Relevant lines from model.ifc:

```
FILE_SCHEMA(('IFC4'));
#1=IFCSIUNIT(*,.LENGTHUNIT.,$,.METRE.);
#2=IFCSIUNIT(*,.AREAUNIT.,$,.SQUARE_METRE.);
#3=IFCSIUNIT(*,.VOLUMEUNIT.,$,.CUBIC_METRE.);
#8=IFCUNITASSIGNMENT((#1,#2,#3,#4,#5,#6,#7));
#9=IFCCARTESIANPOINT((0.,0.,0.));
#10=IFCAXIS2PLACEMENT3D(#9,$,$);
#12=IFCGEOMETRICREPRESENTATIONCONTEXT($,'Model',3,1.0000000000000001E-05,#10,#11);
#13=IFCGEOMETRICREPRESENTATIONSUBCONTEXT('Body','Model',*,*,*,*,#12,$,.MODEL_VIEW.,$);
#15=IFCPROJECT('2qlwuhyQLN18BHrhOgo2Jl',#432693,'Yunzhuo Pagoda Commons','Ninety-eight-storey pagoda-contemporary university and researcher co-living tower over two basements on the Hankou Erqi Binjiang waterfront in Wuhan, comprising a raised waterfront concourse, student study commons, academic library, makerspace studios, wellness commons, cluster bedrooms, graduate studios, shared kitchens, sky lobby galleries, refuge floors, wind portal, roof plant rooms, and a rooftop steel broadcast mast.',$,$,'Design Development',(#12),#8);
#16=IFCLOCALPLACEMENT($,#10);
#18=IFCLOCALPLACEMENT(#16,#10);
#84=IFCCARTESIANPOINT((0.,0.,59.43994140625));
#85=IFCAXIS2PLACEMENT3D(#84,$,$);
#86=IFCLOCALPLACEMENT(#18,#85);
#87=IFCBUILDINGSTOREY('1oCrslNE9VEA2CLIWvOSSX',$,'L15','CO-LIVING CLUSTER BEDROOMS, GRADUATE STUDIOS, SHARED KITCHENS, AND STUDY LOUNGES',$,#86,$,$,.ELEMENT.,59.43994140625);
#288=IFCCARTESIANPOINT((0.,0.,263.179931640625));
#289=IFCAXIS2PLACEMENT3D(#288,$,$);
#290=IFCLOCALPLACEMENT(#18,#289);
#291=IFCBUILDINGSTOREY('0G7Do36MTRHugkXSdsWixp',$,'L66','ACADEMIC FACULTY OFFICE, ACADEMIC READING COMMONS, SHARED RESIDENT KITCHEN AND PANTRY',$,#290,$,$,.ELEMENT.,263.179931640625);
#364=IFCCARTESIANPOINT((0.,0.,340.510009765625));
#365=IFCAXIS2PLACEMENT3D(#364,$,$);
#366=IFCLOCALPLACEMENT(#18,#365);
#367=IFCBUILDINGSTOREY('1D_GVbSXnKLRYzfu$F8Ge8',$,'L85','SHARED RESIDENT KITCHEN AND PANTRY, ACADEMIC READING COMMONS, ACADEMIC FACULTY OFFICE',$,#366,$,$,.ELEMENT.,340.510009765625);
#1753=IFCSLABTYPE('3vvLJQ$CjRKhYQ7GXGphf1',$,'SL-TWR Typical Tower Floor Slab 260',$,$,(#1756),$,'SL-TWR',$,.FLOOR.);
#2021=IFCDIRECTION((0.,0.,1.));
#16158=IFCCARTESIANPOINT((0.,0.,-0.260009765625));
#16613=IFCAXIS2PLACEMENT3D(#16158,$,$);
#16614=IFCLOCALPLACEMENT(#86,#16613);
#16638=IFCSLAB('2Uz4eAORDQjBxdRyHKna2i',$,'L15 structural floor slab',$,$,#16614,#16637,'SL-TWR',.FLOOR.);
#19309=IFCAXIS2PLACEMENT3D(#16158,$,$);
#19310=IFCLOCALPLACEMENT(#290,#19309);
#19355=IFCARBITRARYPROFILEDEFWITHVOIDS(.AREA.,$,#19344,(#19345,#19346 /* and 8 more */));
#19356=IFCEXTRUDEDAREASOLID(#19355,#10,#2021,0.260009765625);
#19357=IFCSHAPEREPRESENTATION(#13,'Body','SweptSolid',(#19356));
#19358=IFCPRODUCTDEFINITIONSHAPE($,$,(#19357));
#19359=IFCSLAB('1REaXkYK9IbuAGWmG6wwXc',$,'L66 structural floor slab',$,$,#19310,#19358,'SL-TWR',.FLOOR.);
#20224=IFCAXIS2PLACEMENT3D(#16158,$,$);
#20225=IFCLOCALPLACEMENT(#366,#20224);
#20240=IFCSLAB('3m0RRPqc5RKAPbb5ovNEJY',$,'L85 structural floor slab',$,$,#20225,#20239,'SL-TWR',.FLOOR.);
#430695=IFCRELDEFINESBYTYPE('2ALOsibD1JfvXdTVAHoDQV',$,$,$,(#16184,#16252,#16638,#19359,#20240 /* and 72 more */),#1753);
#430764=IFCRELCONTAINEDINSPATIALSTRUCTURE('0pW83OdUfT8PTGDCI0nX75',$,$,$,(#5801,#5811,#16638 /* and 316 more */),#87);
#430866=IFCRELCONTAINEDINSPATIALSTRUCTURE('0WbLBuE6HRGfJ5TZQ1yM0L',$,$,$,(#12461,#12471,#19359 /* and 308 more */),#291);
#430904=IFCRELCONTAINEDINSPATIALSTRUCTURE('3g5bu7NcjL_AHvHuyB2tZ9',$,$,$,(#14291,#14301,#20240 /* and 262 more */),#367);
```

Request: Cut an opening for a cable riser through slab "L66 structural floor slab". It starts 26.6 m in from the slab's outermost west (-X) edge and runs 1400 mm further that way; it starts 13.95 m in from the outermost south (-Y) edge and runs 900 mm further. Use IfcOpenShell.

```python
import numpy as np
import ifcopenshell
import ifcopenshell.api.feature
import ifcopenshell.api.geometry
import ifcopenshell.api.root
import ifcopenshell.geom
import ifcopenshell.util.placement
import ifcopenshell.util.representation
import ifcopenshell.util.shape
import ifcopenshell.util.unit

model = ifcopenshell.open("model.ifc")
unit_scale = ifcopenshell.util.unit.calculate_unit_scale(model)
settings = ifcopenshell.geom.settings()


def volume(element):
    """Net volume in cubic metres, openings subtracted."""
    shape = ifcopenshell.geom.create_shape(settings, element)
    return ifcopenshell.util.shape.get_volume(shape.geometry)


slab = model.by_guid("1REaXkYK9IbuAGWmG6wwXc")
before = volume(slab)

# Extent in the slab's own axes, in metres. The edges named are its -X and -Y sides.
slab_shape = ifcopenshell.geom.create_shape(settings, slab)
vertices = ifcopenshell.util.shape.get_vertices(slab_shape.geometry)
x_min, y_min, bottom = vertices.min(axis=0)
top = vertices[:, 2].max()

opening = ifcopenshell.api.root.create_entity(model, ifc_class="IfcOpeningElement", name="Cable riser opening", predefined_type="OPENING")
context = ifcopenshell.util.representation.get_context(model, "Model", "Body", "MODEL_VIEW")
width, depth = 1.4, 0.9
outline = [(0.0, 0.0), (width, 0.0), (width, depth), (0.0, depth), (0.0, 0.0)]
# Overshoot both faces by 50 mm so the cut is clean.
shape = ifcopenshell.api.geometry.add_slab_representation(
    model, context=context, depth=top - bottom + 0.1, polyline=outline
)
ifcopenshell.api.geometry.assign_representation(model, product=opening, representation=shape)

matrix = ifcopenshell.util.placement.get_local_placement(slab.ObjectPlacement)
matrix[:, 3] = matrix @ np.append(np.array([x_min + 26.6, y_min + 13.95, bottom - 0.05]) / unit_scale, 1.0)
ifcopenshell.api.geometry.edit_object_placement(model, product=opening, matrix=matrix, is_si=False)
ifcopenshell.api.feature.add_feature(model, feature=opening, element=slab)

after = volume(slab)

print(f"slab volume {before:.3f} -> {after:.3f} m3")

model.write("model_updated.ifc")
```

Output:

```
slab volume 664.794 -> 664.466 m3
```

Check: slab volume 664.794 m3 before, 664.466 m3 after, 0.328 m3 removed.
